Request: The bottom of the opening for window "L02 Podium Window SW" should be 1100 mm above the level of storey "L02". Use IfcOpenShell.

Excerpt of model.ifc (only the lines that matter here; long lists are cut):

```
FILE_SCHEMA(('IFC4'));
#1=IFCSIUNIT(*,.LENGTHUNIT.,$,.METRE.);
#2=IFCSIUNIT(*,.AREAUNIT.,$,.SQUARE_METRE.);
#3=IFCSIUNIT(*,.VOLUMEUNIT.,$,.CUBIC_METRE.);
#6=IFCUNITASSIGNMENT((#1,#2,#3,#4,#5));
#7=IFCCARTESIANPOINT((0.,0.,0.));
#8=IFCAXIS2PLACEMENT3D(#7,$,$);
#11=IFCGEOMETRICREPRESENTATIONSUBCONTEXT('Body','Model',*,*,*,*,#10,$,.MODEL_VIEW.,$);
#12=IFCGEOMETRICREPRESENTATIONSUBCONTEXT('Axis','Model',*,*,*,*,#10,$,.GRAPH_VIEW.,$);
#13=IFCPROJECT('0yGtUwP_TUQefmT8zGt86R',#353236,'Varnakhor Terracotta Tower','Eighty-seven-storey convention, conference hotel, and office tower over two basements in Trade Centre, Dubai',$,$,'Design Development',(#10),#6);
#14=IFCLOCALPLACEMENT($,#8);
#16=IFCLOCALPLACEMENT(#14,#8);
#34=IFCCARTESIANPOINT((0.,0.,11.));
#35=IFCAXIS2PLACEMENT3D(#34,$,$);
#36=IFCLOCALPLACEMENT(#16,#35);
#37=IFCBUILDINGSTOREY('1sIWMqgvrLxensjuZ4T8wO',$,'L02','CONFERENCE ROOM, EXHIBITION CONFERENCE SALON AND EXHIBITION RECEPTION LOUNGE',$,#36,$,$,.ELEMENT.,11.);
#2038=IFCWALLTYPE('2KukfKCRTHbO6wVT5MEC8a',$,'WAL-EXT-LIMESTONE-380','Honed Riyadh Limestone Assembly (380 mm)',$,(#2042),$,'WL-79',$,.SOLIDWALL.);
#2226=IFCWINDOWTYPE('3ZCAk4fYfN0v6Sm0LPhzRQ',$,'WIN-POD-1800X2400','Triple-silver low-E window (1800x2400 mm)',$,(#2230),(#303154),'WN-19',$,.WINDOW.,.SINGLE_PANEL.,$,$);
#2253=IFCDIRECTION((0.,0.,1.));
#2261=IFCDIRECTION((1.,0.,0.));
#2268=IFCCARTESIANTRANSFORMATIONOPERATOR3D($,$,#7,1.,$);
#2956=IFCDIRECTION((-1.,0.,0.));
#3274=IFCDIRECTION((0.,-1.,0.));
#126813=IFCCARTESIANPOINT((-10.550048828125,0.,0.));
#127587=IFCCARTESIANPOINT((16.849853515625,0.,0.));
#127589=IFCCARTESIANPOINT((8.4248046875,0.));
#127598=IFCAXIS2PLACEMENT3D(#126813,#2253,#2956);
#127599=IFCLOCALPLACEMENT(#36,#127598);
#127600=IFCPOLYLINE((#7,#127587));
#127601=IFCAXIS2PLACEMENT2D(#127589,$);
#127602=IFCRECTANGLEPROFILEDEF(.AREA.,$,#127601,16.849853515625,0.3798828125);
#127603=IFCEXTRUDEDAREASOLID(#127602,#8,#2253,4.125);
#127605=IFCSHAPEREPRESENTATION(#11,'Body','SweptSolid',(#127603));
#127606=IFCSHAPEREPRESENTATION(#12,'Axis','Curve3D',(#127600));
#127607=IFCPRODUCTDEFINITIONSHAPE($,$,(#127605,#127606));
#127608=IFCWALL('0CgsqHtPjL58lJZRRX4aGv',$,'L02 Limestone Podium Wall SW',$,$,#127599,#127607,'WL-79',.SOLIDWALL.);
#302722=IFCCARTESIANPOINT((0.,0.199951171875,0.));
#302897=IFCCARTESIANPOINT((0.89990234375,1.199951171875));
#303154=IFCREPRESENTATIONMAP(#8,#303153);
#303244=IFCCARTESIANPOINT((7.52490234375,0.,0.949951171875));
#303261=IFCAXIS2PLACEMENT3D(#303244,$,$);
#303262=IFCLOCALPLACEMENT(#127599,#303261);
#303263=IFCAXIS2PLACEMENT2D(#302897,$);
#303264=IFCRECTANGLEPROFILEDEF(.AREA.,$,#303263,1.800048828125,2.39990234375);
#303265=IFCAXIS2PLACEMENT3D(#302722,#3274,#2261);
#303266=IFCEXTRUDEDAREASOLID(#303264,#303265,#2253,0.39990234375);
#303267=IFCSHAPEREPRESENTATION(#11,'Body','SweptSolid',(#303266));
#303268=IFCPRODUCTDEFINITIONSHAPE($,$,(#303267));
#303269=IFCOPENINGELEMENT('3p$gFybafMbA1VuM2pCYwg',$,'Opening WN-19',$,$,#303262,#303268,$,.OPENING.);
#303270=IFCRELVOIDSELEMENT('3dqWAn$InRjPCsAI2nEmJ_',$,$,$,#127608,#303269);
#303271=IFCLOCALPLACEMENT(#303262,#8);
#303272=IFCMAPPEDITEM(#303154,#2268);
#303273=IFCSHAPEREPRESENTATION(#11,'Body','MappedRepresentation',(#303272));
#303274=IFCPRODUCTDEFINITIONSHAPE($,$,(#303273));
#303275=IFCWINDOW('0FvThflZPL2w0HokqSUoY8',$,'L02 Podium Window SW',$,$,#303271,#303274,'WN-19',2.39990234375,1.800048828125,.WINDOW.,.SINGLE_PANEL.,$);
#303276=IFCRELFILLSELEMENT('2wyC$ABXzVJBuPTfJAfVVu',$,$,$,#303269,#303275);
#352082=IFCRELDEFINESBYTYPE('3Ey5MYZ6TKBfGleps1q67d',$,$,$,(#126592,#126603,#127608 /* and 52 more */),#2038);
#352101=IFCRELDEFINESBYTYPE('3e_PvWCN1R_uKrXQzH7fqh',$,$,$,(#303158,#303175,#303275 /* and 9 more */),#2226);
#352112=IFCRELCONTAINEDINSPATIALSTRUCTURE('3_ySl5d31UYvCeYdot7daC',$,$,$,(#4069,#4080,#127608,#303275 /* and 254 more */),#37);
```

```python
import numpy as np
import ifcopenshell
import ifcopenshell.api.geometry
import ifcopenshell.geom
import ifcopenshell.util.element
import ifcopenshell.util.placement
import ifcopenshell.util.shape
import ifcopenshell.util.unit

model = ifcopenshell.open("model.ifc")
unit_scale = ifcopenshell.util.unit.calculate_unit_scale(model)

window = model.by_guid("0FvThflZPL2w0HokqSUoY8")
opening = window.FillsVoids[0].RelatingOpeningElement
storey = ifcopenshell.util.element.get_container(window, ifc_class="IfcBuildingStorey")
level = ifcopenshell.util.placement.get_local_placement(storey.ObjectPlacement)[2, 3]

# The opening's origin need not be at the sill, so measure its lowest point.
shape = ifcopenshell.geom.create_shape(ifcopenshell.geom.settings(), opening)
bottom = ifcopenshell.util.shape.get_shape_bottom_elevation(shape, shape.geometry) / unit_scale
dz = level + 1.1 / unit_scale - bottom

shift = np.array([0.0, 0.0, dz])
# The window is placed relative to its opening, so it follows when the opening moves.
matrix = ifcopenshell.util.placement.get_local_placement(opening.ObjectPlacement)
matrix[:3, 3] += shift
ifcopenshell.api.geometry.edit_object_placement(
    model, product=opening, matrix=matrix, is_si=False, should_transform_children=True
)

print(f"moved by {dz * unit_scale:+.3f} m")

model.write("model_updated.ifc")
```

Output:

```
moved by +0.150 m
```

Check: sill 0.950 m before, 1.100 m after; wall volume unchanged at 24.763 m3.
